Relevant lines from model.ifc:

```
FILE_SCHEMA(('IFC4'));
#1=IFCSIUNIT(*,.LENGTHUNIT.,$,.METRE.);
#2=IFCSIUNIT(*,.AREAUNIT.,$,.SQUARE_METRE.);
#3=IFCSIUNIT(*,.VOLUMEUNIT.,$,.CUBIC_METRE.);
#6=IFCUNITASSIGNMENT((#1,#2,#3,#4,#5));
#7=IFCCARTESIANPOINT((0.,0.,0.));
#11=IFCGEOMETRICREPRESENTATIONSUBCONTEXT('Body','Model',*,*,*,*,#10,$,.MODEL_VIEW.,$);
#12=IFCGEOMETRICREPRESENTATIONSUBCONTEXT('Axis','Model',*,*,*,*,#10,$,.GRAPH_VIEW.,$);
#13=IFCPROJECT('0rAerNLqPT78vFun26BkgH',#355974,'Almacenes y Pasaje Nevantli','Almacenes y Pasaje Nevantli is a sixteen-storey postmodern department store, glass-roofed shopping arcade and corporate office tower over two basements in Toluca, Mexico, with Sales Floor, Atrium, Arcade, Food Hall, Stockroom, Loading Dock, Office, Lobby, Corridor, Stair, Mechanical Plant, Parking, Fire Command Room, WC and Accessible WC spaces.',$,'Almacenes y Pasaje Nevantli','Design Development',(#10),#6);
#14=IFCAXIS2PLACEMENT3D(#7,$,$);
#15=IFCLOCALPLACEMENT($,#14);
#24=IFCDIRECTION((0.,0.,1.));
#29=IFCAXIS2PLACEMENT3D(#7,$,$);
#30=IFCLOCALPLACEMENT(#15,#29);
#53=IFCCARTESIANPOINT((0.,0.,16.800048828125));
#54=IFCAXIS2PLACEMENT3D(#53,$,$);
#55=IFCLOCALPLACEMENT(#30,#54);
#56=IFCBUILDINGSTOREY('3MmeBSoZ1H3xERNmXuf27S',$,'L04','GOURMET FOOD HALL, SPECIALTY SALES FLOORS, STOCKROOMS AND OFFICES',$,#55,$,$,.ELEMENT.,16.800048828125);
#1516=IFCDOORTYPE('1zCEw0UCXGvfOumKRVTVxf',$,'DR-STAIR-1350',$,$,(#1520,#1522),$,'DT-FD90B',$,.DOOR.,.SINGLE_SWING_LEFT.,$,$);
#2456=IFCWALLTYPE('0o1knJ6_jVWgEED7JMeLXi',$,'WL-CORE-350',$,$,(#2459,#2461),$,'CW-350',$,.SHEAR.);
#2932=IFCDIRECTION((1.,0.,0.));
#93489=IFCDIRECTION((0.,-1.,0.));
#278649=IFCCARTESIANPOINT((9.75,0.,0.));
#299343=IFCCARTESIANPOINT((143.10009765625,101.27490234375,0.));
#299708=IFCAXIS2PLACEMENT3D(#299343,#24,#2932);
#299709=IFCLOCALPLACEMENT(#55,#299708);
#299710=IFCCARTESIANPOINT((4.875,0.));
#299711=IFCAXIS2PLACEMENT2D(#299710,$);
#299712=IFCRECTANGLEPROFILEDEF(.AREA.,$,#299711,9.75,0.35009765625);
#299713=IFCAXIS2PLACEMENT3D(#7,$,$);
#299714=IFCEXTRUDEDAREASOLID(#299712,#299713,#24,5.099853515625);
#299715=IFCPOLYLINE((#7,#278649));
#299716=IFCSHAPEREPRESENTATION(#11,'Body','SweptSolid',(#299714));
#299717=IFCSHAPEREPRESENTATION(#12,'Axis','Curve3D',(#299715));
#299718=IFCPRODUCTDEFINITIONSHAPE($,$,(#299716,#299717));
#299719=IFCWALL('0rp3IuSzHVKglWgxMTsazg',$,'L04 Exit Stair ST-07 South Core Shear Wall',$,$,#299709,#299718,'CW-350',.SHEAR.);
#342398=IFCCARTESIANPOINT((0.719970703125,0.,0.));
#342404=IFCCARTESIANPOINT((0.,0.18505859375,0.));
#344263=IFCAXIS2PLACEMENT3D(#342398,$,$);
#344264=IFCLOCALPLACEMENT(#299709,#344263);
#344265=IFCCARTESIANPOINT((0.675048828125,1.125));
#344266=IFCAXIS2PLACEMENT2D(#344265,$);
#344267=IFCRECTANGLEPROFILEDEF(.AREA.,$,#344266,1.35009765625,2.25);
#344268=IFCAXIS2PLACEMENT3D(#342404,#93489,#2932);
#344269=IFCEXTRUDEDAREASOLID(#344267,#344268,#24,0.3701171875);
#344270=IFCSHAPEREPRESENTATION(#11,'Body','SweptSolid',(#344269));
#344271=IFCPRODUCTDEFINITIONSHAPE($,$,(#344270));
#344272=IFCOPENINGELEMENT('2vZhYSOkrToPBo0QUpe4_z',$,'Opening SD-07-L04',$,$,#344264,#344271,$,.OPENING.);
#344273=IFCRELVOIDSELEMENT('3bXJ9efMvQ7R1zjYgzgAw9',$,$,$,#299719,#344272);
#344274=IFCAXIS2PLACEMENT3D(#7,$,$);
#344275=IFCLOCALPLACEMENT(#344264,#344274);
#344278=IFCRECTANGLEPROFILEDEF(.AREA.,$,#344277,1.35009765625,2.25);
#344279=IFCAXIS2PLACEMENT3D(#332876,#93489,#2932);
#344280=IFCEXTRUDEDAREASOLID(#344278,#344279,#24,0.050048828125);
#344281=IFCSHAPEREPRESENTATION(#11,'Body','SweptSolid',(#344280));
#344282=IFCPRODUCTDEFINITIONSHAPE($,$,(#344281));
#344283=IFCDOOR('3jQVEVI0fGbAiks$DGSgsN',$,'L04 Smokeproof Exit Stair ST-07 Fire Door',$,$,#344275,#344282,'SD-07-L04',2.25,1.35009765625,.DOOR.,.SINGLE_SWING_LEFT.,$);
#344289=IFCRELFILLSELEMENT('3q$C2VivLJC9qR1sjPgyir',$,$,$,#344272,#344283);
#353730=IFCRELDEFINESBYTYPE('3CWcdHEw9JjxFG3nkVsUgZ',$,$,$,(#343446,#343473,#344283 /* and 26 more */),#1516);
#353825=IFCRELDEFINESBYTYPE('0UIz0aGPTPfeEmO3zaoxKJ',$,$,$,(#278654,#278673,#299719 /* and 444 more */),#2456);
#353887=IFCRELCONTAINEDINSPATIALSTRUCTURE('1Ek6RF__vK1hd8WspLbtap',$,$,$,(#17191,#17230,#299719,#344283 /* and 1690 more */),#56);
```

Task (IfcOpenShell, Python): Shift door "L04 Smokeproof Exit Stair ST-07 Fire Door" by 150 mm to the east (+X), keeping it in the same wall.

```python
import ifcopenshell
import ifcopenshell.api.geometry
import ifcopenshell.util.placement

model = ifcopenshell.open("model.ifc")

door = model.by_guid("3jQVEVI0fGbAiks$DGSgsN")
opening = door.FillsVoids[0].RelatingOpeningElement
wall = opening.VoidsElements[0].RelatingBuildingElement

wall_matrix = ifcopenshell.util.placement.get_local_placement(wall.ObjectPlacement)
shift = wall_matrix[:3, 0] * 0.15
before = ifcopenshell.util.placement.get_local_placement(door.ObjectPlacement)[:3, 3].copy()

# The door is placed relative to its opening, so it follows when the opening moves.
matrix = ifcopenshell.util.placement.get_local_placement(opening.ObjectPlacement)
matrix[:3, 3] += shift
ifcopenshell.api.geometry.edit_object_placement(
    model, product=opening, matrix=matrix, is_si=False, should_transform_children=True
)

after = ifcopenshell.util.placement.get_local_placement(door.ObjectPlacement)[:3, 3]
print("door moved by", (after - before).round(3) + 0.0)

model.write("model-out.ifc")
```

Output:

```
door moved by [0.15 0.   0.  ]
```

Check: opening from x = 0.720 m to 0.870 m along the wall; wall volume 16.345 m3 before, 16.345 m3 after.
